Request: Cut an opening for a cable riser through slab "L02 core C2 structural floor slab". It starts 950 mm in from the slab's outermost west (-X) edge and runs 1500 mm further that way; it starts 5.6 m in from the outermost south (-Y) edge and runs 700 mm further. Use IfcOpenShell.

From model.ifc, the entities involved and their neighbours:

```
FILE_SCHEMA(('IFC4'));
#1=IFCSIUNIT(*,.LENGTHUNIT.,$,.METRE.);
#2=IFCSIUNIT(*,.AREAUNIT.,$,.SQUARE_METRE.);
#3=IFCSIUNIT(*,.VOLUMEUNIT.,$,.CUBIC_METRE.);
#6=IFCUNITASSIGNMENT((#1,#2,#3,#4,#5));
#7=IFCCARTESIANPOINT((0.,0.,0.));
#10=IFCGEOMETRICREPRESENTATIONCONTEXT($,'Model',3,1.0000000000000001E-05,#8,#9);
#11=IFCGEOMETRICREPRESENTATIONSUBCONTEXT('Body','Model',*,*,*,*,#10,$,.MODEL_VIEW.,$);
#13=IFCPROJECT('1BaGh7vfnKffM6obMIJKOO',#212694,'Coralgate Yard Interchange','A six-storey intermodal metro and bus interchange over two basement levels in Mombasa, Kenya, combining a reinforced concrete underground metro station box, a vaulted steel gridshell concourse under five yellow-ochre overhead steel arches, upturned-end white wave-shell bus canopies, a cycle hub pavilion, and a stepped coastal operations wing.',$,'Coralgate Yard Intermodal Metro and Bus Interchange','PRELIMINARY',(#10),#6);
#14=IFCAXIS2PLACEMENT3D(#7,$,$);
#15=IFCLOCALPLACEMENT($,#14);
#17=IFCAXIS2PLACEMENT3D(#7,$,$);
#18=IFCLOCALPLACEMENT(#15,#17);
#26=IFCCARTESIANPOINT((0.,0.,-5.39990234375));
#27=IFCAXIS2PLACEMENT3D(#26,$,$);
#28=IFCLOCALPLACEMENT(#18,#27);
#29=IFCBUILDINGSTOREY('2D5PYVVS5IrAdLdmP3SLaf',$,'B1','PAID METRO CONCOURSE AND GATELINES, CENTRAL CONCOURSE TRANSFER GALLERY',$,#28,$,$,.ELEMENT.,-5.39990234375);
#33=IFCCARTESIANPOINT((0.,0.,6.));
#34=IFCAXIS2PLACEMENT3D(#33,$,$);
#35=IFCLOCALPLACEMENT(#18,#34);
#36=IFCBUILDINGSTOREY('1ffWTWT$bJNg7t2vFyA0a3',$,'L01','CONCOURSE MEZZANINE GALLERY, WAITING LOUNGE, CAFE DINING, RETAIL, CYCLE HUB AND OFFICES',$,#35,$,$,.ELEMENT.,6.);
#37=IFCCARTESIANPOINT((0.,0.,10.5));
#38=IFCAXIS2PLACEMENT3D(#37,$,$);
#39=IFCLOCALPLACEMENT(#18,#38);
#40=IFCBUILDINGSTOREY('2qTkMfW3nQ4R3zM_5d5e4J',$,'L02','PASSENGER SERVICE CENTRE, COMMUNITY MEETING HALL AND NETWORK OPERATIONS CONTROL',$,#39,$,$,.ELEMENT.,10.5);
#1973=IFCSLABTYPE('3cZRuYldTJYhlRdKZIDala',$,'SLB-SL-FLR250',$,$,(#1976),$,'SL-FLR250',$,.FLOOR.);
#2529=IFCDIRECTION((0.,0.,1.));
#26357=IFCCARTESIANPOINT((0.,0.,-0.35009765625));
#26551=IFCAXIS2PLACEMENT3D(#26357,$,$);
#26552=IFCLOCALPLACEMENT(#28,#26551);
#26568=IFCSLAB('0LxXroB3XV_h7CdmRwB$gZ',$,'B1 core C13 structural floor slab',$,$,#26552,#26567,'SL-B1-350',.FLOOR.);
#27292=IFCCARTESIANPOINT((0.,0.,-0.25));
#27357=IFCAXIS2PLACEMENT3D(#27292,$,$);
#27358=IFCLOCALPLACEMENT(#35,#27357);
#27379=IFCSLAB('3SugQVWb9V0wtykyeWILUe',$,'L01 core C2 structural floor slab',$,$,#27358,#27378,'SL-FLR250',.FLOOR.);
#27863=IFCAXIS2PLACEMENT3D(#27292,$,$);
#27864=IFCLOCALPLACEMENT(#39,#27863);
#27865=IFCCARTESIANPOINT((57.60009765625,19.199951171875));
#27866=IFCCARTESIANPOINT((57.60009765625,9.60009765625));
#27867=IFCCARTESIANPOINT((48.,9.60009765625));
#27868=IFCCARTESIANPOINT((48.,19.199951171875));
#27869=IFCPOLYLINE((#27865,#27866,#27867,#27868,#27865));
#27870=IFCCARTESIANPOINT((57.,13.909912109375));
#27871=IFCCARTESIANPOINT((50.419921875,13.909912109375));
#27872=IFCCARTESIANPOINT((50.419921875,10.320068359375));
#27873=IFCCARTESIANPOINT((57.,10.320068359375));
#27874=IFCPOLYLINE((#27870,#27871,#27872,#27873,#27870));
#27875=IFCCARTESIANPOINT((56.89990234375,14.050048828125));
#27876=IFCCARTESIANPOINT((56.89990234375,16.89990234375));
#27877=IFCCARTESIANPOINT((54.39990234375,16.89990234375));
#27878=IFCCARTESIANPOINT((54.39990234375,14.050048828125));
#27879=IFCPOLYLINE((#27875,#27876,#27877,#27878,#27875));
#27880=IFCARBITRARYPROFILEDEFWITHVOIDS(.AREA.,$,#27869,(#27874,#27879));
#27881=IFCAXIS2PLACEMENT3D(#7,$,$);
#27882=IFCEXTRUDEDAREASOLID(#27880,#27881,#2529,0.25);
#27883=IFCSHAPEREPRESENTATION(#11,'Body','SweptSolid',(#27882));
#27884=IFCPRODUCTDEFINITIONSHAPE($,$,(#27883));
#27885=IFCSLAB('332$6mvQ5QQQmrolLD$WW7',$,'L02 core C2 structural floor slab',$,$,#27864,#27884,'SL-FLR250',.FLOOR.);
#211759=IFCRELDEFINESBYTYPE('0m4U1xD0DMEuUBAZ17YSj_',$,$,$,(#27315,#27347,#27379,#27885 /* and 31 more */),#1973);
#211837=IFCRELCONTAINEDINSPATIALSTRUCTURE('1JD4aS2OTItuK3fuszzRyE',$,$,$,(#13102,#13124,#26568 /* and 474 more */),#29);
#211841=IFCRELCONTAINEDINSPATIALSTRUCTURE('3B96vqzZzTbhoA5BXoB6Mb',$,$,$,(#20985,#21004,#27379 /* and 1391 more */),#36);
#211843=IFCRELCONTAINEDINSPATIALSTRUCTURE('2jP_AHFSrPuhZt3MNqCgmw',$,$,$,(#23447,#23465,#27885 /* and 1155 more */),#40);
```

```python
import numpy as np
import ifcopenshell
import ifcopenshell.api.feature
import ifcopenshell.api.geometry
import ifcopenshell.api.root
import ifcopenshell.geom
import ifcopenshell.util.placement
import ifcopenshell.util.representation
import ifcopenshell.util.shape
import ifcopenshell.util.unit

model = ifcopenshell.open("model.ifc")
unit_scale = ifcopenshell.util.unit.calculate_unit_scale(model)
settings = ifcopenshell.geom.settings()


def volume(element):
    """Net volume in cubic metres, openings subtracted."""
    shape = ifcopenshell.geom.create_shape(settings, element)
    return ifcopenshell.util.shape.get_volume(shape.geometry)


slab = model.by_guid("332$6mvQ5QQQmrolLD$WW7")
before = volume(slab)

# Extent in the slab's own axes, in metres. The edges named are its -X and -Y sides.
slab_shape = ifcopenshell.geom.create_shape(settings, slab)
vertices = ifcopenshell.util.shape.get_vertices(slab_shape.geometry)
x_min, y_min, bottom = vertices.min(axis=0)
top = vertices[:, 2].max()

opening = ifcopenshell.api.root.create_entity(model, ifc_class="IfcOpeningElement", name="Cable riser opening", predefined_type="OPENING")
context = ifcopenshell.util.representation.get_context(model, "Model", "Body", "MODEL_VIEW")
width, depth = 1.5, 0.7
outline = [(0.0, 0.0), (width, 0.0), (width, depth), (0.0, depth), (0.0, 0.0)]
# Overshoot both faces by 50 mm so the cut is clean.
shape = ifcopenshell.api.geometry.add_slab_representation(
    model, context=context, depth=top - bottom + 0.1, polyline=outline
)
ifcopenshell.api.geometry.assign_representation(model, product=opening, representation=shape)

matrix = ifcopenshell.util.placement.get_local_placement(slab.ObjectPlacement)
matrix[:, 3] = matrix @ np.append(np.array([x_min + 0.95, y_min + 5.6, bottom - 0.05]) / unit_scale, 1.0)
ifcopenshell.api.geometry.edit_object_placement(model, product=opening, matrix=matrix, is_si=False)
ifcopenshell.api.feature.add_feature(model, feature=opening, element=slab)

after = volume(slab)

print(f"slab volume {before:.3f} -> {after:.3f} m3")

model.write("model_v2.ifc")
```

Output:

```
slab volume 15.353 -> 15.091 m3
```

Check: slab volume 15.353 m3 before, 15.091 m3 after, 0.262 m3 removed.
